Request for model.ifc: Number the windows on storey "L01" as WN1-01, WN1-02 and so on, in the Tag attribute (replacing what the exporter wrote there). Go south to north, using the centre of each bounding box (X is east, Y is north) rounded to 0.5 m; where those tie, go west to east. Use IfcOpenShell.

First a look at what the model holds.

```python
import ifcopenshell
import ifcopenshell.util.element
import ifcopenshell.util.placement

model = ifcopenshell.open("model.ifc")
print(model.schema)
storey = next(s for s in model.by_type("IfcBuildingStorey") if s.Name == "L01")
windows = [e for e in ifcopenshell.util.element.get_decomposition(storey) if e.is_a("IfcWindow")]
for e in sorted(windows, key=lambda e: e.id()):
    origin = ifcopenshell.util.placement.get_local_placement(e.ObjectPlacement)[:3, 3]
    print(e.id(), e.Tag, e.Name, origin.round(2) + 0.0, sep=" | ")
```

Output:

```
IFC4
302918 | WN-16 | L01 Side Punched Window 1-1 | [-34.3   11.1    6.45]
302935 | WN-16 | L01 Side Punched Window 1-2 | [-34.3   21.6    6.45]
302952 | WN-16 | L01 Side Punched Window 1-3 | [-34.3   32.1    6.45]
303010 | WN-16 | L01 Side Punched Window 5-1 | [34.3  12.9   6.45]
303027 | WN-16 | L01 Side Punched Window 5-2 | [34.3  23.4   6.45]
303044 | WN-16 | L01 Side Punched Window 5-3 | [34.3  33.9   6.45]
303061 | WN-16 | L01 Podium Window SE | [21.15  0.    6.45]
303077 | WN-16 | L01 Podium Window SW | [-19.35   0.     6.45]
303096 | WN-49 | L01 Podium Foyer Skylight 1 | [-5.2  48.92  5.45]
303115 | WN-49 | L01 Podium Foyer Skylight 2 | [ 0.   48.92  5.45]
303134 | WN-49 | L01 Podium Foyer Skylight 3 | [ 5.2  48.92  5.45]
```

```python
import ifcopenshell
import ifcopenshell.geom
import ifcopenshell.util.element
import ifcopenshell.util.shape

model = ifcopenshell.open("model.ifc")
settings = ifcopenshell.geom.settings()
settings.set("use-world-coords", True)


def centre(element):
    shape = ifcopenshell.geom.create_shape(settings, element)
    return ifcopenshell.util.shape.get_bbox_centroid(shape.geometry)


storey = next(s for s in model.by_type("IfcBuildingStorey") if s.Name == "L01")
windows = [e for e in ifcopenshell.util.element.get_decomposition(storey) if e.is_a("IfcWindow")]

# Insertion points can sit at a corner or the storey origin, so sort by the geometry (in metres).
centres = {e: centre(e) for e in windows}
windows.sort(key=lambda e: (round(centres[e][1] / 0.5), centres[e][0]))

for i, e in enumerate(windows, start=1):
    number = f"WN1-{i:02d}"
    e.Tag = number
    print(e.id(), number)

model.write("model-out.ifc")
```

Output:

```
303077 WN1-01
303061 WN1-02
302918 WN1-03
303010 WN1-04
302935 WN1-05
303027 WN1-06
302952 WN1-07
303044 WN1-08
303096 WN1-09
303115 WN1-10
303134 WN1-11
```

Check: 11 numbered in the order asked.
